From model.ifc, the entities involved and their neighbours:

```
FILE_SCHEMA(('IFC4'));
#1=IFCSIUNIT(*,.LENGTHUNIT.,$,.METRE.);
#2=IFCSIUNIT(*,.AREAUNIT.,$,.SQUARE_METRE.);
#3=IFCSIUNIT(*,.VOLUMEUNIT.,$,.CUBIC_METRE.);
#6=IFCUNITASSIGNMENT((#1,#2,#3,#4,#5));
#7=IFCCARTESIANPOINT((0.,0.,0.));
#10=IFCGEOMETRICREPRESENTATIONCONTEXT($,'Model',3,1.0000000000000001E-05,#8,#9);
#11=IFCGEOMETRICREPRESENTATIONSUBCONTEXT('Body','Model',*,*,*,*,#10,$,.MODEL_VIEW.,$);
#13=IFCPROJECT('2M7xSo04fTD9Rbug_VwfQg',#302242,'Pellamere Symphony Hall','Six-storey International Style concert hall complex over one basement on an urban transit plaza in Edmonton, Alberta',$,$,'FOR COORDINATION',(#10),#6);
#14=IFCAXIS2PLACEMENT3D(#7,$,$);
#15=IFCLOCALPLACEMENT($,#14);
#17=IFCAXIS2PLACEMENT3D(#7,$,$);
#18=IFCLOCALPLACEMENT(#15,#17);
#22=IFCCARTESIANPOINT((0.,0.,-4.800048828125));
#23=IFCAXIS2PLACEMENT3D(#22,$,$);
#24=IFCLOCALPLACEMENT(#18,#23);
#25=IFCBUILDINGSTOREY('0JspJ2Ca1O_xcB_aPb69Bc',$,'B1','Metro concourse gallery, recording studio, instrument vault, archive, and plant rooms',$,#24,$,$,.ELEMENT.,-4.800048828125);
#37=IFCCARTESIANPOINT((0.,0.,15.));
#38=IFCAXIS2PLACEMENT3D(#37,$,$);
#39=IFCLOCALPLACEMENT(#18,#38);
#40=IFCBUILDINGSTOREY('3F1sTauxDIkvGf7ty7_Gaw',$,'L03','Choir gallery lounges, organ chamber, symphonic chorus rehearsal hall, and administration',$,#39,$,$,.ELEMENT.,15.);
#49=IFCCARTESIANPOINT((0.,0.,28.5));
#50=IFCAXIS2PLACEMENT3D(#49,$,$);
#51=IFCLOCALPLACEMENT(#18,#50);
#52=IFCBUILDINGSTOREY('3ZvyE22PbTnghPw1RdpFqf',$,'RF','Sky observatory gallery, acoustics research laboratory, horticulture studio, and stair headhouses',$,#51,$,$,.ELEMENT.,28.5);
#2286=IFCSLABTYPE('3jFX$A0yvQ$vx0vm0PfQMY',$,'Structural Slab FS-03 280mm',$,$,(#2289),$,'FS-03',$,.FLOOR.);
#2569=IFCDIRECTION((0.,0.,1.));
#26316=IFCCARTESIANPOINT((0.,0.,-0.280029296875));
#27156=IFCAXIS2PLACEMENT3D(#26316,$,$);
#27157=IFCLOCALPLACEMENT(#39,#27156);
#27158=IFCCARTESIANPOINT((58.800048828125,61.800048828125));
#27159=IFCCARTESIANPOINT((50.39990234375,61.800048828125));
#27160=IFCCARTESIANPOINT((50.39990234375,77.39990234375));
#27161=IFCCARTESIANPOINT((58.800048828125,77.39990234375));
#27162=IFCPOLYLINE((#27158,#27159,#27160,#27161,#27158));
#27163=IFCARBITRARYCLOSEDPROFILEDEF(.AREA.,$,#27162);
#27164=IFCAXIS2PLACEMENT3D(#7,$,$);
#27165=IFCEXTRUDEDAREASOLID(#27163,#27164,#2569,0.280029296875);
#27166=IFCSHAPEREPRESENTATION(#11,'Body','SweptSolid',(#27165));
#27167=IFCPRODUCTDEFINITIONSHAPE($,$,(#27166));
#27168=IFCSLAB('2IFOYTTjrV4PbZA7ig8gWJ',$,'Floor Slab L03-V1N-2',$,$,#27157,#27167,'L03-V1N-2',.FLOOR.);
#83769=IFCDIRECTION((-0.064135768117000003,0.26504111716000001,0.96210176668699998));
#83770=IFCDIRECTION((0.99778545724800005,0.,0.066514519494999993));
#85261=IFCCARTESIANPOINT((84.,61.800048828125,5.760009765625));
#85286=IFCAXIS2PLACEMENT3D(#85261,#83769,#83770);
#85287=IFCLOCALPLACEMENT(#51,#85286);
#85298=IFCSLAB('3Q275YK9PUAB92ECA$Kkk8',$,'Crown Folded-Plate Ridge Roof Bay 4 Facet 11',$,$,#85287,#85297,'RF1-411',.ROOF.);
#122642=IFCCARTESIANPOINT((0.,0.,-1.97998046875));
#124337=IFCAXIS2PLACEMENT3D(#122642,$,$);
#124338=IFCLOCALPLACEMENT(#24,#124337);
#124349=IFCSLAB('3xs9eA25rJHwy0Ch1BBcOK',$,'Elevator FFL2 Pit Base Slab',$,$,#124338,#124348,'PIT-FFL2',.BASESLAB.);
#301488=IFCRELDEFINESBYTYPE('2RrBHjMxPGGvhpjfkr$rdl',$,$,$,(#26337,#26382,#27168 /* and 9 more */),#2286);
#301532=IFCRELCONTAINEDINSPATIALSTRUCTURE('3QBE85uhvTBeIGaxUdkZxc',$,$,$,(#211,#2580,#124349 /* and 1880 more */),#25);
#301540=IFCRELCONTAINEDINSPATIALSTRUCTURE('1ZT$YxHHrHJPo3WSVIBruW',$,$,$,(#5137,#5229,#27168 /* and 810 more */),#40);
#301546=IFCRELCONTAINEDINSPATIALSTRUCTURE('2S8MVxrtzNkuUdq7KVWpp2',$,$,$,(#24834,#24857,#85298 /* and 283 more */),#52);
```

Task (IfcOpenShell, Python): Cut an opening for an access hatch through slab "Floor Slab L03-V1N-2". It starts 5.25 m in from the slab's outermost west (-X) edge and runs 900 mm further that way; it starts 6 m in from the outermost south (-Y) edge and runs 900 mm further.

```python
import numpy as np
import ifcopenshell
import ifcopenshell.api.feature
import ifcopenshell.api.geometry
import ifcopenshell.api.root
import ifcopenshell.geom
import ifcopenshell.util.placement
import ifcopenshell.util.representation
import ifcopenshell.util.shape
import ifcopenshell.util.unit

model = ifcopenshell.open("model.ifc")
unit_scale = ifcopenshell.util.unit.calculate_unit_scale(model)
settings = ifcopenshell.geom.settings()


def volume(element):
    """Net volume in cubic metres, openings subtracted."""
    shape = ifcopenshell.geom.create_shape(settings, element)
    return ifcopenshell.util.shape.get_volume(shape.geometry)


slab = model.by_guid("2IFOYTTjrV4PbZA7ig8gWJ")
before = volume(slab)

# Extent in the slab's own axes, in metres. The edges named are its -X and -Y sides.
slab_shape = ifcopenshell.geom.create_shape(settings, slab)
vertices = ifcopenshell.util.shape.get_vertices(slab_shape.geometry)
x_min, y_min, bottom = vertices.min(axis=0)
top = vertices[:, 2].max()

opening = ifcopenshell.api.root.create_entity(model, ifc_class="IfcOpeningElement", name="Access hatch opening", predefined_type="OPENING")
context = ifcopenshell.util.representation.get_context(model, "Model", "Body", "MODEL_VIEW")
width, depth = 0.9, 0.9
outline = [(0.0, 0.0), (width, 0.0), (width, depth), (0.0, depth), (0.0, 0.0)]
# Overshoot both faces by 50 mm so the cut is clean.
shape = ifcopenshell.api.geometry.add_slab_representation(
    model, context=context, depth=top - bottom + 0.1, polyline=outline
)
ifcopenshell.api.geometry.assign_representation(model, product=opening, representation=shape)

matrix = ifcopenshell.util.placement.get_local_placement(slab.ObjectPlacement)
matrix[:, 3] = matrix @ np.append(np.array([x_min + 5.25, y_min + 6, bottom - 0.05]) / unit_scale, 1.0)
ifcopenshell.api.geometry.edit_object_placement(model, product=opening, matrix=matrix, is_si=False)
ifcopenshell.api.feature.add_feature(model, feature=opening, element=slab)

after = volume(slab)

print(f"slab volume {before:.3f} -> {after:.3f} m3")

model.write("model_updated.ifc")
```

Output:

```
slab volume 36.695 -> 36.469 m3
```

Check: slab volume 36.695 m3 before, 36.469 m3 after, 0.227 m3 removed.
